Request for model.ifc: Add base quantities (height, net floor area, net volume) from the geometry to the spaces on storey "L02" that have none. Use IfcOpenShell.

First a look at what the model holds.

```python
import ifcopenshell
import ifcopenshell.util.element
import ifcopenshell.util.unit

model = ifcopenshell.open("model.ifc")
print(model.schema)
for unit_type in ("LENGTHUNIT", "AREAUNIT", "VOLUMEUNIT"):
    print(unit_type, ifcopenshell.util.unit.calculate_unit_scale(model, unit_type))
storey = next(s for s in model.by_type("IfcBuildingStorey") if s.Name == "L02")
spaces = [e for e in ifcopenshell.util.element.get_decomposition(storey) if e.is_a("IfcSpace")]
for e in sorted(spaces, key=lambda e: e.id()):
    print(e.id(), e.is_a(), e.Name, list(ifcopenshell.util.element.get_psets(e, qtos_only=True)), sep=" | ")
```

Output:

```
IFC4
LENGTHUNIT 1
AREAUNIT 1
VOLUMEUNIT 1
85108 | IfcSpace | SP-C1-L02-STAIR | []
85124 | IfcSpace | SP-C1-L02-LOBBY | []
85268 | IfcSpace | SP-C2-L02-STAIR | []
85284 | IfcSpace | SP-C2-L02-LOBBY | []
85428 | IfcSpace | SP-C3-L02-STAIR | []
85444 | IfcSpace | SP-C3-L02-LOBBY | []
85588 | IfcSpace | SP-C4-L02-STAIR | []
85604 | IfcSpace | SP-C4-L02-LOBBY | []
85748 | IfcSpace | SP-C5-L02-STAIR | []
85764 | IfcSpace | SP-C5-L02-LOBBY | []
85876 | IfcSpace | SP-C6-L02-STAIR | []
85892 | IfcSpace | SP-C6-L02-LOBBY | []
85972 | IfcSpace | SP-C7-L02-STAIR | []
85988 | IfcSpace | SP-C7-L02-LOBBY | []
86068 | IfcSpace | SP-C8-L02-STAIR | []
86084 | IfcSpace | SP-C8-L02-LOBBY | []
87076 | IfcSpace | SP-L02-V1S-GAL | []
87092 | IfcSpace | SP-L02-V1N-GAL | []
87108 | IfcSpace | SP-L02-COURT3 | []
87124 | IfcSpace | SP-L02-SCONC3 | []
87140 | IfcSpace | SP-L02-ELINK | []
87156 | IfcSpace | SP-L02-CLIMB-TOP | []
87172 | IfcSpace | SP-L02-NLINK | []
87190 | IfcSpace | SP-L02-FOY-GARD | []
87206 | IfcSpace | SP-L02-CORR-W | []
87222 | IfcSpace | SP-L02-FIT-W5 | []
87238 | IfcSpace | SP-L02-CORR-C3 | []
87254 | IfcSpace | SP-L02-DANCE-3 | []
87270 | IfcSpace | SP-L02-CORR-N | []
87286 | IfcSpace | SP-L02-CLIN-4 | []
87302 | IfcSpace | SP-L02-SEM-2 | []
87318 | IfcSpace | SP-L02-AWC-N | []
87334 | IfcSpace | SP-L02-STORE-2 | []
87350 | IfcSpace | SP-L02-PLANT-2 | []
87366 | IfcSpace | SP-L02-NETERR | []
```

```python
import ifcopenshell
import ifcopenshell.api.pset
import ifcopenshell.geom
import ifcopenshell.util.element
import ifcopenshell.util.shape
import ifcopenshell.util.unit

model = ifcopenshell.open("model.ifc")
unit_scale = ifcopenshell.util.unit.calculate_unit_scale(model)
area_scale = ifcopenshell.util.unit.calculate_unit_scale(model, "AREAUNIT")
volume_scale = ifcopenshell.util.unit.calculate_unit_scale(model, "VOLUMEUNIT")
settings = ifcopenshell.geom.settings()

storey = next(s for s in model.by_type("IfcBuildingStorey") if s.Name == "L02")
spaces = [e for e in ifcopenshell.util.element.get_decomposition(storey) if e.is_a("IfcSpace")]

for e in sorted(spaces, key=lambda e: e.id()):
    if ifcopenshell.util.element.get_psets(e, qtos_only=True, should_inherit=False):
        continue
    # Geometry comes back in metres, in the element's own axes.
    shape = ifcopenshell.geom.create_shape(settings, e)
    values = {
        "Height": ifcopenshell.util.shape.get_z(shape.geometry) / unit_scale,
        "NetFloorArea": ifcopenshell.util.shape.get_footprint_area(shape.geometry) / area_scale,
        "NetVolume": ifcopenshell.util.shape.get_volume(shape.geometry) / volume_scale,
    }
    qto = ifcopenshell.api.pset.add_qto(model, product=e, name="Qto_SpaceBaseQuantities")
    ifcopenshell.api.pset.edit_qto(model, qto=qto, properties=values)
    print(e.id(), {k: round(v, 3) for k, v in values.items()})

model.write("model_v2.ifc")
```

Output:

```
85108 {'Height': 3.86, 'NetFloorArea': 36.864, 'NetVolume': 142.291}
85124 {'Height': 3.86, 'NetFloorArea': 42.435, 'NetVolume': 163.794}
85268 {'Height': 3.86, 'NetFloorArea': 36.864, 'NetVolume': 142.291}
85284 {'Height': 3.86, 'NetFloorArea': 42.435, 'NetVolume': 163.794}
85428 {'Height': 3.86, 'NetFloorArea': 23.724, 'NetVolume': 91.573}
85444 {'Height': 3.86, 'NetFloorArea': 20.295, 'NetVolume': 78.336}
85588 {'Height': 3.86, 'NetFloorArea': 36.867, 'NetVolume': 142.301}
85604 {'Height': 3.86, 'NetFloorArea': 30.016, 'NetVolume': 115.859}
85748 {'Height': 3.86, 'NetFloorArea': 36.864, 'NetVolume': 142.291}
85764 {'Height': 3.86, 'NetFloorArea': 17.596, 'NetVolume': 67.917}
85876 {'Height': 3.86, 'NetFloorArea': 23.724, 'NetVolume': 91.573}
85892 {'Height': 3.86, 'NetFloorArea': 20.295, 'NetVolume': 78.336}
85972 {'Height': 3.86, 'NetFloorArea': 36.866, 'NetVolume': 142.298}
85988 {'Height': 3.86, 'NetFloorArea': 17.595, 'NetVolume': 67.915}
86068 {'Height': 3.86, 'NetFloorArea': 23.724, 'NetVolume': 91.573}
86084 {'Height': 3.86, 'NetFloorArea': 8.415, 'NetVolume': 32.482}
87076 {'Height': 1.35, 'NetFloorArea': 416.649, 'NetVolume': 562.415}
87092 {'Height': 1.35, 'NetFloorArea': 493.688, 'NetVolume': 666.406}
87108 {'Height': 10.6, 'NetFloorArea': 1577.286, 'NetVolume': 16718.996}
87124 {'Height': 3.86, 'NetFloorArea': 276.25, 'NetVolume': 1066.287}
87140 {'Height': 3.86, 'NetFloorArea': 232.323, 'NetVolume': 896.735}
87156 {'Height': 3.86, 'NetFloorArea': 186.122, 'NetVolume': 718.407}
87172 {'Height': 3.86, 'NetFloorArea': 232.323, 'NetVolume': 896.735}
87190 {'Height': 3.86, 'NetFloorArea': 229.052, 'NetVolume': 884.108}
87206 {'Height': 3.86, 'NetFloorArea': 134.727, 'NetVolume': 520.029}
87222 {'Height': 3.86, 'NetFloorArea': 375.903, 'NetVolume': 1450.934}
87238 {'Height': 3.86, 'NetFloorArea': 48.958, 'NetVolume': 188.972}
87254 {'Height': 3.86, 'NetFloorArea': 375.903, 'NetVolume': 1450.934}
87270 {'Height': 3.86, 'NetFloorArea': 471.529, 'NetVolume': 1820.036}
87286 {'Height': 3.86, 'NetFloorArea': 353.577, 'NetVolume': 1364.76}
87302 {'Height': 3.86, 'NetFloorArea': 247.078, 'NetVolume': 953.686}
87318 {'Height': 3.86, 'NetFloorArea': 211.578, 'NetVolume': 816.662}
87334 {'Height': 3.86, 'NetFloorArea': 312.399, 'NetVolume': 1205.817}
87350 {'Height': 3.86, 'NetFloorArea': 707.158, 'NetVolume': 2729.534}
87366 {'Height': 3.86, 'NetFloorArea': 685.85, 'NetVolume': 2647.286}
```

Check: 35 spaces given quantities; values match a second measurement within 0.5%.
